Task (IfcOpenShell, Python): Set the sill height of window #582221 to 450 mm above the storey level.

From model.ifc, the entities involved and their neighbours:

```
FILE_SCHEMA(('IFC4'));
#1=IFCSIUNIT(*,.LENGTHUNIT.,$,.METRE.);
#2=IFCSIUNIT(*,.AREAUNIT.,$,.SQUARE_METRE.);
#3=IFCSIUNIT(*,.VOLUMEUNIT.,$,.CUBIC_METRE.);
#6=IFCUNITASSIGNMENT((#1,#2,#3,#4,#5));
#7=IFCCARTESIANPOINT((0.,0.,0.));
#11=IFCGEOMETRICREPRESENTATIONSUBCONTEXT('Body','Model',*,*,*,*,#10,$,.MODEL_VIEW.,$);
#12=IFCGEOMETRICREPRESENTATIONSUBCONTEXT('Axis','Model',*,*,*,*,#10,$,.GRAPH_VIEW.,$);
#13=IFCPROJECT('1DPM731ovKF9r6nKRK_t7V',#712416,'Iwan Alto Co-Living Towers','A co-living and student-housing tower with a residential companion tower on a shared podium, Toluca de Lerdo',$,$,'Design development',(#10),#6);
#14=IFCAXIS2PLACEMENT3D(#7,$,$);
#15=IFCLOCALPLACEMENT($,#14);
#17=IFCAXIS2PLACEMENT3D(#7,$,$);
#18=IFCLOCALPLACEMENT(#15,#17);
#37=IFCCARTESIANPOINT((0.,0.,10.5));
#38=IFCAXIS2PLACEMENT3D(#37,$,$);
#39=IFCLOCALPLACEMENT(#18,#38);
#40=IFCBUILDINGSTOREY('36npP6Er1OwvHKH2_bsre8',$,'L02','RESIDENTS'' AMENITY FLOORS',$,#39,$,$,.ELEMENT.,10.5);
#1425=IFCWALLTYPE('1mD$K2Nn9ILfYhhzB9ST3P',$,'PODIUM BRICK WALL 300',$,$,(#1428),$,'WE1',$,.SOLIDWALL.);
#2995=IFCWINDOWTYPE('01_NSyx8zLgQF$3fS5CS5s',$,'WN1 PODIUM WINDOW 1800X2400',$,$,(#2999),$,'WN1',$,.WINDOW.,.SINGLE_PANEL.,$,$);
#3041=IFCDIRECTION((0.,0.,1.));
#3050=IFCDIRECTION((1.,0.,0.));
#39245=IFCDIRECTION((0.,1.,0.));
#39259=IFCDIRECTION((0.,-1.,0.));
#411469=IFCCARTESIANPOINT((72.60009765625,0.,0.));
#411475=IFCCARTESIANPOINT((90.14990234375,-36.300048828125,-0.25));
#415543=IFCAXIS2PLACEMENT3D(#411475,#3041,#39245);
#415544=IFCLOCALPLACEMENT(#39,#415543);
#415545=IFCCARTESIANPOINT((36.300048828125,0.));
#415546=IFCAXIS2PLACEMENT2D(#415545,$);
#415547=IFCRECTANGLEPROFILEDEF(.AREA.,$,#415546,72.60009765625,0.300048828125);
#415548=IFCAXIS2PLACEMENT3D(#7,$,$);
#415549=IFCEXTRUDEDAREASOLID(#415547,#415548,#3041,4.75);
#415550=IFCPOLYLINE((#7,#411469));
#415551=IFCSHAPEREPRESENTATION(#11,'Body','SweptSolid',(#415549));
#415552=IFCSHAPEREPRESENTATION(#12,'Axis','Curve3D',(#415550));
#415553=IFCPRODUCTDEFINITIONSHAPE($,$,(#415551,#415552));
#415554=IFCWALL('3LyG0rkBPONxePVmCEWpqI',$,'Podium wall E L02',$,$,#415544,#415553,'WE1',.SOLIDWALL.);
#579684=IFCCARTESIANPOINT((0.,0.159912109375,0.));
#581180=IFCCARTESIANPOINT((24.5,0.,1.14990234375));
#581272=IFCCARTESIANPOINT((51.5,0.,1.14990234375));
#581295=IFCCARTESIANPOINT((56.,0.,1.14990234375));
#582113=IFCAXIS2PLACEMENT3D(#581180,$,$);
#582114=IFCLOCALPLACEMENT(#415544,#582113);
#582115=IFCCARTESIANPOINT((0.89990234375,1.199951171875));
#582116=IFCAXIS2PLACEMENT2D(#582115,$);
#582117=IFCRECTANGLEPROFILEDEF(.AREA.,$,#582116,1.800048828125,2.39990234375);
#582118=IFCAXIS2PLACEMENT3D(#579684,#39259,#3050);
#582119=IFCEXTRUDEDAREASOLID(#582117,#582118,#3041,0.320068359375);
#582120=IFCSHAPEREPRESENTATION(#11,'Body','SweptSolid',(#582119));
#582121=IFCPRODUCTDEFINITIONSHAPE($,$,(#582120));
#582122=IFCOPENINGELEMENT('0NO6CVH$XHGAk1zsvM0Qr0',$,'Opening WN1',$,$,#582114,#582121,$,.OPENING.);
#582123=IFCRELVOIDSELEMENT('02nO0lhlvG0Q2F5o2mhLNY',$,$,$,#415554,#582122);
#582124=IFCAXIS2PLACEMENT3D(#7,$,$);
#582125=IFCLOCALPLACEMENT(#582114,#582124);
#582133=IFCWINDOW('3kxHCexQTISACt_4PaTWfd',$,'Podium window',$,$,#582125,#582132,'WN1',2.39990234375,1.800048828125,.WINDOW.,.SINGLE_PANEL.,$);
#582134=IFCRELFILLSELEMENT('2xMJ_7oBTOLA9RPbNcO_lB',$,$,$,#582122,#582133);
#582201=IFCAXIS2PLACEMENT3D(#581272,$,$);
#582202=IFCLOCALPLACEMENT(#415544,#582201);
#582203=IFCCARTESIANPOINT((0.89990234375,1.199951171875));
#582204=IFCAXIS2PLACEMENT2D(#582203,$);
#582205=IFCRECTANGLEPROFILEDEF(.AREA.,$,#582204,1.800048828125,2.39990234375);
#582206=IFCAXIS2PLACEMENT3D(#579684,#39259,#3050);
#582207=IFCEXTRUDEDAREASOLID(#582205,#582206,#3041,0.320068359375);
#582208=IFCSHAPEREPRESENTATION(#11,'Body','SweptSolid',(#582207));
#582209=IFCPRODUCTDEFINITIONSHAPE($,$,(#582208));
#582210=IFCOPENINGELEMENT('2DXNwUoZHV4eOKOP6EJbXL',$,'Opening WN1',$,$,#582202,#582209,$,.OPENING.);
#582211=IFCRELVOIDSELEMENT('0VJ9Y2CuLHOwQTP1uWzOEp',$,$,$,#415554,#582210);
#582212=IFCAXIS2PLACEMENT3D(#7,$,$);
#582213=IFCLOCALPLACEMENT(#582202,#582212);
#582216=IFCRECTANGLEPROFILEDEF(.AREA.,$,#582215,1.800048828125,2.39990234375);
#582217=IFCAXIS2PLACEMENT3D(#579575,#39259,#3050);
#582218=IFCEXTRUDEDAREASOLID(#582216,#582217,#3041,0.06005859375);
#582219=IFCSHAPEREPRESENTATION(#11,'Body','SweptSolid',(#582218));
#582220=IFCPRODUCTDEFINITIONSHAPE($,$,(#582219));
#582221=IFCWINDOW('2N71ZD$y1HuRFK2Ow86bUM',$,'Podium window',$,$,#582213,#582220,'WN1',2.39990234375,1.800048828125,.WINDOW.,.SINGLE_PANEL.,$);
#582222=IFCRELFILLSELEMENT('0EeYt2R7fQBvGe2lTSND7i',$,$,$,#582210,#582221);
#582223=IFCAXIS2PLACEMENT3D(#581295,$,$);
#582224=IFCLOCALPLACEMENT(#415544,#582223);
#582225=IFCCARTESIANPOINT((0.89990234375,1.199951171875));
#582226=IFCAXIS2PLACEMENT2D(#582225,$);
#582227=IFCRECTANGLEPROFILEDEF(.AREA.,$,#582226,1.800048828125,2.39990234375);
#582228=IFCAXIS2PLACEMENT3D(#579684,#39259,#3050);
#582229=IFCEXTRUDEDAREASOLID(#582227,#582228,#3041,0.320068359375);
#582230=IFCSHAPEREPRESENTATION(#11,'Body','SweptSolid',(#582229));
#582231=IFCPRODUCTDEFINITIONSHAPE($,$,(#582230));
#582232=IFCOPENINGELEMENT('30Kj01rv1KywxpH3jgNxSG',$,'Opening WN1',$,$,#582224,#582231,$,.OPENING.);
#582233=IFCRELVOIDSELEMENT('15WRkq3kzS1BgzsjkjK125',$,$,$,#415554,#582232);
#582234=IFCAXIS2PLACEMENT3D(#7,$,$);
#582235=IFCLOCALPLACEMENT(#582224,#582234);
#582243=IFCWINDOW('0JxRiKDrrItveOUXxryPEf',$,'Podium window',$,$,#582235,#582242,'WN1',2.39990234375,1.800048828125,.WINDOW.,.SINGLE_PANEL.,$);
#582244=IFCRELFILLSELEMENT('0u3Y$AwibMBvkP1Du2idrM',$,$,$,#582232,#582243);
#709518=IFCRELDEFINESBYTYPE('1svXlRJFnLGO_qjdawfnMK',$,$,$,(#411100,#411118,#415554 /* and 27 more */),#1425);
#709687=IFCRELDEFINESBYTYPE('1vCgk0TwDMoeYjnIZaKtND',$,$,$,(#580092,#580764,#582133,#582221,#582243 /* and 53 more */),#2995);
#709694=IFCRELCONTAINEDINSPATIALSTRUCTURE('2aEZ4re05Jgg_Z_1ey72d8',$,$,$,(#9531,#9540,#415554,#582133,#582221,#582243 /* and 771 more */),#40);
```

```python
import numpy as np
import ifcopenshell
import ifcopenshell.api.geometry
import ifcopenshell.geom
import ifcopenshell.util.element
import ifcopenshell.util.placement
import ifcopenshell.util.shape
import ifcopenshell.util.unit

model = ifcopenshell.open("model.ifc")
unit_scale = ifcopenshell.util.unit.calculate_unit_scale(model)

window = model.by_guid("2N71ZD$y1HuRFK2Ow86bUM")
opening = window.FillsVoids[0].RelatingOpeningElement
storey = ifcopenshell.util.element.get_container(window, ifc_class="IfcBuildingStorey")
level = ifcopenshell.util.placement.get_local_placement(storey.ObjectPlacement)[2, 3]

# The opening's origin need not be at the sill, so measure its lowest point.
shape = ifcopenshell.geom.create_shape(ifcopenshell.geom.settings(), opening)
bottom = ifcopenshell.util.shape.get_shape_bottom_elevation(shape, shape.geometry) / unit_scale
dz = level + 0.45 / unit_scale - bottom

shift = np.array([0.0, 0.0, dz])
# The window is placed relative to its opening, so it follows when the opening moves.
matrix = ifcopenshell.util.placement.get_local_placement(opening.ObjectPlacement)
matrix[:3, 3] += shift
ifcopenshell.api.geometry.edit_object_placement(
    model, product=opening, matrix=matrix, is_si=False, should_transform_children=True
)

print(f"moved by {dz * unit_scale:+.3f} m")

model.write("model_updated.ifc")
```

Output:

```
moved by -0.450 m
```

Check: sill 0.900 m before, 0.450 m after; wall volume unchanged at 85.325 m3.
